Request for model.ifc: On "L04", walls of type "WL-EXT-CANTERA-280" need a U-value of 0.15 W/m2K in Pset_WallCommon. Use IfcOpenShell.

First a look at what the model holds.

```python
import ifcopenshell
import ifcopenshell.util.element

model = ifcopenshell.open("model.ifc")
print(model.schema)
storey = next(s for s in model.by_type("IfcBuildingStorey") if s.Name == "L04")
walls = [e for e in ifcopenshell.util.element.get_decomposition(storey) if e.is_a("IfcWall")]
seen = {}
for e in walls:
    element_type = ifcopenshell.util.element.get_type(e)
    key = (element_type.Name if element_type != e and element_type else None, ifcopenshell.util.element.get_pset(e, "Pset_WallCommon", "ThermalTransmittance"))
    seen[key] = seen.get(key, 0) + 1
for (name, value), count in sorted(seen.items(), key=str):
    print(count, "x", name, "|", value)
```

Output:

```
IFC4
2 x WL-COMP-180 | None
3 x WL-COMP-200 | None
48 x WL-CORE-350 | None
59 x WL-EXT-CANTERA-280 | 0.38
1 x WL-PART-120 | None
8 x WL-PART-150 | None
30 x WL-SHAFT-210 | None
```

```python
import ifcopenshell
import ifcopenshell.api.pset
import ifcopenshell.util.element

model = ifcopenshell.open("model.ifc")

storey = next(s for s in model.by_type("IfcBuildingStorey") if s.Name == "L04")
walls = [e for e in ifcopenshell.util.element.get_decomposition(storey) if e.is_a("IfcWall")]

count = 0
for e in walls:
    element_type = ifcopenshell.util.element.get_type(e)
    if element_type in (None, e) or element_type.Name != "WL-EXT-CANTERA-280":
        continue
    # add_pset returns the element's existing set when there is one.
    pset = ifcopenshell.api.pset.add_pset(model, product=e, name="Pset_WallCommon")
    ifcopenshell.api.pset.edit_pset(model, pset=pset, properties={"ThermalTransmittance": 0.15})
    count += 1

print(count, "walls updated")

model.write("model_v2.ifc")
```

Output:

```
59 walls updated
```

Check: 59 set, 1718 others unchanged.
